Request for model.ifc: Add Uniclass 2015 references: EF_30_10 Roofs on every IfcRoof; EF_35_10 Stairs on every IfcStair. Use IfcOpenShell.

First a look at what the model holds.

```python
import ifcopenshell

model = ifcopenshell.open("model.ifc")
print(model.schema)
print("classifications:", [c.Name for c in model.by_type("IfcClassification")])
for ifc_class in ("IfcDoor", "IfcRoof", "IfcStair", "IfcWall", "IfcWindow"):
    print(ifc_class, len(model.by_type(ifc_class)))
```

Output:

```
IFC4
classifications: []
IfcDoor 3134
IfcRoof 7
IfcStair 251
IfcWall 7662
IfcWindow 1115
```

```python
import ifcopenshell
import ifcopenshell.api.classification

model = ifcopenshell.open("model.ifc")

system = ifcopenshell.api.classification.add_classification(model, classification="Uniclass 2015")

codes = {
    "IfcRoof": ("EF_30_10", "Roofs"),
    "IfcStair": ("EF_35_10", "Stairs"),
}
for ifc_class, (code, name) in codes.items():
    products = model.by_type(ifc_class)
    ifcopenshell.api.classification.add_reference(
        model, products=products, classification=system, identification=code, name=name
    )
    print(code, len(products))

model.write("model_updated.ifc")
```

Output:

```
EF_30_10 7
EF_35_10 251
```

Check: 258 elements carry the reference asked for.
